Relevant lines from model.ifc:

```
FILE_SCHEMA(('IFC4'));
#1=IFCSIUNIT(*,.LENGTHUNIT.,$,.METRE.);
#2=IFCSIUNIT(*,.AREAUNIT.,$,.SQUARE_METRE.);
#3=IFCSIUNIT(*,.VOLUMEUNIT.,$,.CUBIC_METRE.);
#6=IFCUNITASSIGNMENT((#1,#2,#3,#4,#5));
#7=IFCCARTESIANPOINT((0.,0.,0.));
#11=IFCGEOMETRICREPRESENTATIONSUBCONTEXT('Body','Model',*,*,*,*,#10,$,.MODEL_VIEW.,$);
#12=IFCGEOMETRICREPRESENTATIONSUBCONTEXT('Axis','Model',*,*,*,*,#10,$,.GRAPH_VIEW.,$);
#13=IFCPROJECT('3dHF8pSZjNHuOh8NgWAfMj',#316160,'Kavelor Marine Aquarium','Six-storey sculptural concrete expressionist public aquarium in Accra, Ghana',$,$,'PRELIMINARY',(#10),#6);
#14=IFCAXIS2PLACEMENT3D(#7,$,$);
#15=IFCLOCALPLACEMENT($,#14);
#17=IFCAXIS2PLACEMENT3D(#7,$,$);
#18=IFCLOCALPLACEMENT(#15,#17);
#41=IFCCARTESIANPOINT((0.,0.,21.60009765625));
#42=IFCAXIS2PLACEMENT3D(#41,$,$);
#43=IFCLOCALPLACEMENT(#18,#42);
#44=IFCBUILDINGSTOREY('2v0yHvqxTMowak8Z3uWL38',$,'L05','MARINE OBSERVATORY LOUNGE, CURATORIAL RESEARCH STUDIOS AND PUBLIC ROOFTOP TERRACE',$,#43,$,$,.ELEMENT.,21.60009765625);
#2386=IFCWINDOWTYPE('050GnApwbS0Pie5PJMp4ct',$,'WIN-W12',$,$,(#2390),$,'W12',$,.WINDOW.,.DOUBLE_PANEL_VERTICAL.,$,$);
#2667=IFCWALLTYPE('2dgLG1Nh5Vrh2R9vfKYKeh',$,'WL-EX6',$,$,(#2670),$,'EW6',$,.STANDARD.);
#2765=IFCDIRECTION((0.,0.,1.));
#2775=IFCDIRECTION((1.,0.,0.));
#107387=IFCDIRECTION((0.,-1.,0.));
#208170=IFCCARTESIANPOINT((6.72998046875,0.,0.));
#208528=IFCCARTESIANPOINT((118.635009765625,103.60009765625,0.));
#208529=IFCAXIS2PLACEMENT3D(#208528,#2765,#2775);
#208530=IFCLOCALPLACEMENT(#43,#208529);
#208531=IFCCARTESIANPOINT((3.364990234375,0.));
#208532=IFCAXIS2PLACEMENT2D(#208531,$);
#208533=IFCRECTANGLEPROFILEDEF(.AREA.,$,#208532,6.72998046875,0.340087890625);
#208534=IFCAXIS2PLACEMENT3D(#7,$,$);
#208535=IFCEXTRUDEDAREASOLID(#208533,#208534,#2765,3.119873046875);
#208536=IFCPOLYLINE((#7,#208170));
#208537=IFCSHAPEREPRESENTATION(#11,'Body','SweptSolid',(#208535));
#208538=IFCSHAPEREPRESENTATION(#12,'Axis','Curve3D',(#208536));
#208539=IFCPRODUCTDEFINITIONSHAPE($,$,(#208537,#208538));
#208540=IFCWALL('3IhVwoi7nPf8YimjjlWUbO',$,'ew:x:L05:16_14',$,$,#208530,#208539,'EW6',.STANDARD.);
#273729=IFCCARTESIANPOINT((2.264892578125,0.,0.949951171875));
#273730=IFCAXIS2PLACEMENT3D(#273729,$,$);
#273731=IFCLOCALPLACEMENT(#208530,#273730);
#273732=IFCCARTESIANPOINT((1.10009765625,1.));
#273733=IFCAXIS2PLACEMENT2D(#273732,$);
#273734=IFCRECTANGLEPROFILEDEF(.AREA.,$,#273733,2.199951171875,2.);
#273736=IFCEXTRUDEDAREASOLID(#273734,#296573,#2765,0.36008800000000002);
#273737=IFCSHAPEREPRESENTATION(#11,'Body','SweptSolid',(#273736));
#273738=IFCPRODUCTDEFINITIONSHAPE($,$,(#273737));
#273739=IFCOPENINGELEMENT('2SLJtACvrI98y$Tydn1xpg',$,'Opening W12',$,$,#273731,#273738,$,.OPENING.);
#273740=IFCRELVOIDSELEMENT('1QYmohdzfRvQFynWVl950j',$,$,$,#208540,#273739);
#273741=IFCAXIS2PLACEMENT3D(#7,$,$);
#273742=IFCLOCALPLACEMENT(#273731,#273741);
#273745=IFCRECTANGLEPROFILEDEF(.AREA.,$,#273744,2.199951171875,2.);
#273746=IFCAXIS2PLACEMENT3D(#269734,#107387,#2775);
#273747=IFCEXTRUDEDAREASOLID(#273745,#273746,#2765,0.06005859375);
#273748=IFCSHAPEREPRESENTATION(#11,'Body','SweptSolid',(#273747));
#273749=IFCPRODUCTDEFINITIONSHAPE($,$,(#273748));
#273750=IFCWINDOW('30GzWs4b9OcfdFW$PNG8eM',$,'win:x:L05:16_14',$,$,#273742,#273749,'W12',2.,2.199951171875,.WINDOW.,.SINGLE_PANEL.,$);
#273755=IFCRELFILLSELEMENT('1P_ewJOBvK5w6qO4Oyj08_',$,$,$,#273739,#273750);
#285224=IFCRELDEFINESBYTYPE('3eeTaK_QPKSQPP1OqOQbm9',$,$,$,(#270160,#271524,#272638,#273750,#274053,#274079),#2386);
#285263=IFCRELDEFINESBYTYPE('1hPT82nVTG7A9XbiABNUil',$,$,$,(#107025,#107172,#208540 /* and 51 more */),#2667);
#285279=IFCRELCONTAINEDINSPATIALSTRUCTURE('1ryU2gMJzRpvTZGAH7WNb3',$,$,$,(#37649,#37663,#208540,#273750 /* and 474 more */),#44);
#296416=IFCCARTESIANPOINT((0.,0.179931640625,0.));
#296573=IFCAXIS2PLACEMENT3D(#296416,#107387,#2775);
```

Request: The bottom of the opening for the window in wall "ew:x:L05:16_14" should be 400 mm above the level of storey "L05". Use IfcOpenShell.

```python
import numpy as np
import ifcopenshell
import ifcopenshell.api.geometry
import ifcopenshell.geom
import ifcopenshell.util.element
import ifcopenshell.util.placement
import ifcopenshell.util.shape
import ifcopenshell.util.unit

model = ifcopenshell.open("model.ifc")
unit_scale = ifcopenshell.util.unit.calculate_unit_scale(model)

window = model.by_id(273750)
opening = window.FillsVoids[0].RelatingOpeningElement
storey = ifcopenshell.util.element.get_container(window, ifc_class="IfcBuildingStorey")
level = ifcopenshell.util.placement.get_local_placement(storey.ObjectPlacement)[2, 3]

# The opening's origin need not be at the sill, so measure its lowest point.
shape = ifcopenshell.geom.create_shape(ifcopenshell.geom.settings(), opening)
bottom = ifcopenshell.util.shape.get_shape_bottom_elevation(shape, shape.geometry) / unit_scale
dz = level + 0.4 / unit_scale - bottom

shift = np.array([0.0, 0.0, dz])
# The window is placed relative to its opening, so it follows when the opening moves.
matrix = ifcopenshell.util.placement.get_local_placement(opening.ObjectPlacement)
matrix[:3, 3] += shift
ifcopenshell.api.geometry.edit_object_placement(
    model, product=opening, matrix=matrix, is_si=False, should_transform_children=True
)

print(f"moved by {dz * unit_scale:+.3f} m")

model.write("model_v2.ifc")
```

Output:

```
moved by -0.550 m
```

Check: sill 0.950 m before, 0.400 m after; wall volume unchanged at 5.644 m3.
